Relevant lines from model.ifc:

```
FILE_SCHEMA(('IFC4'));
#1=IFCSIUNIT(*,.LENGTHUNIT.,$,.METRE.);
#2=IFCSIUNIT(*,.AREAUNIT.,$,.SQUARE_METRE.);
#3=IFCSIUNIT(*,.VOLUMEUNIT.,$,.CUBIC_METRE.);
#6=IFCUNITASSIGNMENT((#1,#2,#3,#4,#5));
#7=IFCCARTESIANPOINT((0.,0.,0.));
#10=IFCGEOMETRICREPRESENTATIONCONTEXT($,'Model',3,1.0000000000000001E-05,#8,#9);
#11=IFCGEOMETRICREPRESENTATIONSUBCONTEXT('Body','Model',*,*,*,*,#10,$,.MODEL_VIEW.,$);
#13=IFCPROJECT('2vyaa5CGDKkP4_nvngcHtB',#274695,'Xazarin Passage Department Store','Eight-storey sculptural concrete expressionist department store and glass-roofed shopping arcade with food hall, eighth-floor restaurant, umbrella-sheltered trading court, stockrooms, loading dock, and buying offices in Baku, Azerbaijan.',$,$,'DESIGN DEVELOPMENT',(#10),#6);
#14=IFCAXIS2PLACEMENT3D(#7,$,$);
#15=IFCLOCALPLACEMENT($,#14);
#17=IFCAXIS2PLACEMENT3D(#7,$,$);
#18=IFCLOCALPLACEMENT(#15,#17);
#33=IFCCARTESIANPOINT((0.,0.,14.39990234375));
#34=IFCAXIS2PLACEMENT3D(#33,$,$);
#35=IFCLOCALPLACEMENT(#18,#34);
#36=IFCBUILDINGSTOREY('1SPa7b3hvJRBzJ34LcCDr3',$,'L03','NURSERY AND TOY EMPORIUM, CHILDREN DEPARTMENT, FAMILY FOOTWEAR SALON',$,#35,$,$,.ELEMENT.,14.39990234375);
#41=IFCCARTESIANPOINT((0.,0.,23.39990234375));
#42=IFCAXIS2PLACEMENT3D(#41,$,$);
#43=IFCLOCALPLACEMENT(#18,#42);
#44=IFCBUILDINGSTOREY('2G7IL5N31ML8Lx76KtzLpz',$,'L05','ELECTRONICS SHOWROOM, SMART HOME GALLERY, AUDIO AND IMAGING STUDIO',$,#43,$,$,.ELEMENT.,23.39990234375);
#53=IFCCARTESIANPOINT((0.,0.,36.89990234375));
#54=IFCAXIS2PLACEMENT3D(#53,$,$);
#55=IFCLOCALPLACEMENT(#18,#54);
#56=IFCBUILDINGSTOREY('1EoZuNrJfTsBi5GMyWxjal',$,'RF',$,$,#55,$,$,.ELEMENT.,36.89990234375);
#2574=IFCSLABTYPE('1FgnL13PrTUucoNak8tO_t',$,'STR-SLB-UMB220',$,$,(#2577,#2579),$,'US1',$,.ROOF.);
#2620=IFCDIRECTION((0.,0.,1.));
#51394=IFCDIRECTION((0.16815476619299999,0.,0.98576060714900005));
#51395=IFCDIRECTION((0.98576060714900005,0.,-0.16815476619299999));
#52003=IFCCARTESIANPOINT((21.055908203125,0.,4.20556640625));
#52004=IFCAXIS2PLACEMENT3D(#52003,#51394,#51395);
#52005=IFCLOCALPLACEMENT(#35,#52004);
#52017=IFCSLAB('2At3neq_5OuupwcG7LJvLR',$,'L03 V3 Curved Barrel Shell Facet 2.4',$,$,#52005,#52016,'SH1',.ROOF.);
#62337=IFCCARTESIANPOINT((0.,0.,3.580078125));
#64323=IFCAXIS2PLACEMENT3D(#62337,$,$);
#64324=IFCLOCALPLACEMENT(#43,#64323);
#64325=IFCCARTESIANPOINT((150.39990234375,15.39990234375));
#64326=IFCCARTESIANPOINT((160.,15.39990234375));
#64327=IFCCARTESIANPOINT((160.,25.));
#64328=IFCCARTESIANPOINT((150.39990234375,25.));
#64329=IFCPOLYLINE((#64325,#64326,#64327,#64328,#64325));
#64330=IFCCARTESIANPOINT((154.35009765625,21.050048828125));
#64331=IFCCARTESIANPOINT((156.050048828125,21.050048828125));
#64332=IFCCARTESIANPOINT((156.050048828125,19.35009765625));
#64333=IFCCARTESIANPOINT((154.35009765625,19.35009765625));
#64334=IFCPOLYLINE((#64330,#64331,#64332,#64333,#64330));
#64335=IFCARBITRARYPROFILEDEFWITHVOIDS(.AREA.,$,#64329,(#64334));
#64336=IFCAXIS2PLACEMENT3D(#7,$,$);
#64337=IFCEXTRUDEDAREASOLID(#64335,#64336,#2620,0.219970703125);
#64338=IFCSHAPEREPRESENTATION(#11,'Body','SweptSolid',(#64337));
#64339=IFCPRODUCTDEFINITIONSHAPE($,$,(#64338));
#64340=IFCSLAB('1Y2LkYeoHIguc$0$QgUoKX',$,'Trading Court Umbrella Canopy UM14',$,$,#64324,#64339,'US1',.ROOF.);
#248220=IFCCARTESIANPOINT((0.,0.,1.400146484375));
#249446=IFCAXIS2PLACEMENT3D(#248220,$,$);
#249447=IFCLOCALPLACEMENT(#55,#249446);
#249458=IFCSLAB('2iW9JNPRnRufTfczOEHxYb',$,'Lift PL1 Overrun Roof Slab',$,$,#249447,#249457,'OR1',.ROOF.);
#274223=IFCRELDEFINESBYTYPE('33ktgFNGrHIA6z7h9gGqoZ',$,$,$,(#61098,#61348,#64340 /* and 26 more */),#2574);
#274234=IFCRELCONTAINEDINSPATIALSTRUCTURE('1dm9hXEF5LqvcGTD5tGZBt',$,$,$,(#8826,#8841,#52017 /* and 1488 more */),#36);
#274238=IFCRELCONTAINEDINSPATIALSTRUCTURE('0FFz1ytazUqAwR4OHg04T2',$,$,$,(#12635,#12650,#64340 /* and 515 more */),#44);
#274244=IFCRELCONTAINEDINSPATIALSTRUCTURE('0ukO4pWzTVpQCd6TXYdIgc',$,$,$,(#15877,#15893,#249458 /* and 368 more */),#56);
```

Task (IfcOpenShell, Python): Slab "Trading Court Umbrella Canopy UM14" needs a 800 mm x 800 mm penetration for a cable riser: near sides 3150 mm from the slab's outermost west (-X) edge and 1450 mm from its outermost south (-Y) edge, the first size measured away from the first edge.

```python
import numpy as np
import ifcopenshell
import ifcopenshell.api.feature
import ifcopenshell.api.geometry
import ifcopenshell.api.root
import ifcopenshell.geom
import ifcopenshell.util.placement
import ifcopenshell.util.representation
import ifcopenshell.util.shape
import ifcopenshell.util.unit

model = ifcopenshell.open("model.ifc")
unit_scale = ifcopenshell.util.unit.calculate_unit_scale(model)
settings = ifcopenshell.geom.settings()


def volume(element):
    """Net volume in cubic metres, openings subtracted."""
    shape = ifcopenshell.geom.create_shape(settings, element)
    return ifcopenshell.util.shape.get_volume(shape.geometry)


slab = model.by_id(64340)
before = volume(slab)

# Extent in the slab's own axes, in metres. The edges named are its -X and -Y sides.
slab_shape = ifcopenshell.geom.create_shape(settings, slab)
vertices = ifcopenshell.util.shape.get_vertices(slab_shape.geometry)
x_min, y_min, bottom = vertices.min(axis=0)
top = vertices[:, 2].max()

opening = ifcopenshell.api.root.create_entity(model, ifc_class="IfcOpeningElement", name="Cable riser opening", predefined_type="OPENING")
context = ifcopenshell.util.representation.get_context(model, "Model", "Body", "MODEL_VIEW")
width, depth = 0.8, 0.8
outline = [(0.0, 0.0), (width, 0.0), (width, depth), (0.0, depth), (0.0, 0.0)]
# Overshoot both faces by 50 mm so the cut is clean.
shape = ifcopenshell.api.geometry.add_slab_representation(
    model, context=context, depth=top - bottom + 0.1, polyline=outline
)
ifcopenshell.api.geometry.assign_representation(model, product=opening, representation=shape)

matrix = ifcopenshell.util.placement.get_local_placement(slab.ObjectPlacement)
matrix[:, 3] = matrix @ np.append(np.array([x_min + 3.15, y_min + 1.45, bottom - 0.05]) / unit_scale, 1.0)
ifcopenshell.api.geometry.edit_object_placement(model, product=opening, matrix=matrix, is_si=False)
ifcopenshell.api.feature.add_feature(model, feature=opening, element=slab)

after = volume(slab)

print(f"slab volume {before:.3f} -> {after:.3f} m3")

model.write("model_edited.ifc")
```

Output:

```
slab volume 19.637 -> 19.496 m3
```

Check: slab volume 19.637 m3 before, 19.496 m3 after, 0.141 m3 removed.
